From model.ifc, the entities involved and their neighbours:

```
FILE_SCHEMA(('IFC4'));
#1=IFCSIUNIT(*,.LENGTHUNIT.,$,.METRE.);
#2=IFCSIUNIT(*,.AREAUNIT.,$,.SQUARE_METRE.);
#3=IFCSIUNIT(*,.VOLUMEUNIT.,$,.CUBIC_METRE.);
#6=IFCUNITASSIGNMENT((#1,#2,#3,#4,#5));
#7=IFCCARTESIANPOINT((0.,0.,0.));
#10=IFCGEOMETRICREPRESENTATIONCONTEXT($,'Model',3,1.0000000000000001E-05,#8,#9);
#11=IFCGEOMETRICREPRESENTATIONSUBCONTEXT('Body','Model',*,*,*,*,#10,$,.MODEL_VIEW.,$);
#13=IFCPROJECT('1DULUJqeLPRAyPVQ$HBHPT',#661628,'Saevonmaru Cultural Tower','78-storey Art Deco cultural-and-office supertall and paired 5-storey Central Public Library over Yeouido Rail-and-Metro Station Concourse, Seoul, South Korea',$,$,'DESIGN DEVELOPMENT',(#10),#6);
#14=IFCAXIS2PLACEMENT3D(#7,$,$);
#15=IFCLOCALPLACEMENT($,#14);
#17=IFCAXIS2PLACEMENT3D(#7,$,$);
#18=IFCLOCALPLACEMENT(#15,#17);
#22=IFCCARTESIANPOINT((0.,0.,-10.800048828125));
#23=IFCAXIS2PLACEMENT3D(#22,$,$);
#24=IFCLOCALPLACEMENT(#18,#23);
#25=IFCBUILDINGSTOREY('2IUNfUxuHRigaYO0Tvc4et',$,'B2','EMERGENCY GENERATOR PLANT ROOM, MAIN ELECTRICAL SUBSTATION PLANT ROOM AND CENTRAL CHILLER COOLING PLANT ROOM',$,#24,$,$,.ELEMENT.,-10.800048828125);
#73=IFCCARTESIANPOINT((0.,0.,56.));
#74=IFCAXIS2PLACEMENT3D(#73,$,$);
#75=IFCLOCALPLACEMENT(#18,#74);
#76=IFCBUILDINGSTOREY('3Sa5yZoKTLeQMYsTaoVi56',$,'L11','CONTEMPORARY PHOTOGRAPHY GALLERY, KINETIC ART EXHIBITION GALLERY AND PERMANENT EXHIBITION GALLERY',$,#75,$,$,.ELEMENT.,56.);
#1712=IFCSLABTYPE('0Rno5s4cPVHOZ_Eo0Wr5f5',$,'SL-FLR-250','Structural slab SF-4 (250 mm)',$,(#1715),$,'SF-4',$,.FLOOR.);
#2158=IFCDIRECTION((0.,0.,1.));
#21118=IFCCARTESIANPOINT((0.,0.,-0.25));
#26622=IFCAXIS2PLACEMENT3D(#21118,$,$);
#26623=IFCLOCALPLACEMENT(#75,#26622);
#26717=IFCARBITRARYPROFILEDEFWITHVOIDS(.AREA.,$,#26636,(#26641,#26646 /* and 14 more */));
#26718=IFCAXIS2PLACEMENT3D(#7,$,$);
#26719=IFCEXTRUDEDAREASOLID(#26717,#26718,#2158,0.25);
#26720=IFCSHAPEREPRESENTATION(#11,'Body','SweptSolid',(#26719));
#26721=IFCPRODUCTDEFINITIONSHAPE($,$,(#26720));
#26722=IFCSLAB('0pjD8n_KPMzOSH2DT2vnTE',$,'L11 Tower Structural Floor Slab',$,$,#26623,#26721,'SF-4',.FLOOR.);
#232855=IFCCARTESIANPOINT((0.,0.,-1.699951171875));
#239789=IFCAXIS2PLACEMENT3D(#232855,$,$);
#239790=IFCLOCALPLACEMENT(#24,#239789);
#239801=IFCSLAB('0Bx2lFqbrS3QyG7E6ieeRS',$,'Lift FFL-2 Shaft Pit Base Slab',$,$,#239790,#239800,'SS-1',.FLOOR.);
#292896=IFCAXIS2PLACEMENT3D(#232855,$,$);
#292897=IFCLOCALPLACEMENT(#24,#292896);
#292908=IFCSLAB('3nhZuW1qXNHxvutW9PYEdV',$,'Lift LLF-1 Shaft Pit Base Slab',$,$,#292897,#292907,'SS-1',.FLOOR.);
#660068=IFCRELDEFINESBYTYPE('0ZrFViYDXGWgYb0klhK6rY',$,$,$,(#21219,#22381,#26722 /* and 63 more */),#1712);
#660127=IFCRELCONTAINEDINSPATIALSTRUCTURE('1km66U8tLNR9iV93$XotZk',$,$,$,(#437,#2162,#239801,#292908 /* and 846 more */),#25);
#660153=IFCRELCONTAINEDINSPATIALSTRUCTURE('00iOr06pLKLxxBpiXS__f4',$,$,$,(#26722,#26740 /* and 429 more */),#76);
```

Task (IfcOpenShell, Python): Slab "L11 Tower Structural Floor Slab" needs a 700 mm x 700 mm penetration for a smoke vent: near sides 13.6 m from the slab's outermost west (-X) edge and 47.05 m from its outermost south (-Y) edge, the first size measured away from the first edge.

```python
import numpy as np
import ifcopenshell
import ifcopenshell.api.feature
import ifcopenshell.api.geometry
import ifcopenshell.api.root
import ifcopenshell.geom
import ifcopenshell.util.placement
import ifcopenshell.util.representation
import ifcopenshell.util.shape
import ifcopenshell.util.unit

model = ifcopenshell.open("model.ifc")
unit_scale = ifcopenshell.util.unit.calculate_unit_scale(model)
settings = ifcopenshell.geom.settings()


def volume(element):
    """Net volume in cubic metres, openings subtracted."""
    shape = ifcopenshell.geom.create_shape(settings, element)
    return ifcopenshell.util.shape.get_volume(shape.geometry)


slab = model.by_guid("0pjD8n_KPMzOSH2DT2vnTE")
before = volume(slab)

# Extent in the slab's own axes, in metres. The edges named are its -X and -Y sides.
slab_shape = ifcopenshell.geom.create_shape(settings, slab)
vertices = ifcopenshell.util.shape.get_vertices(slab_shape.geometry)
x_min, y_min, bottom = vertices.min(axis=0)
top = vertices[:, 2].max()

opening = ifcopenshell.api.root.create_entity(model, ifc_class="IfcOpeningElement", name="Smoke vent opening", predefined_type="OPENING")
context = ifcopenshell.util.representation.get_context(model, "Model", "Body", "MODEL_VIEW")
width, depth = 0.7, 0.7
outline = [(0.0, 0.0), (width, 0.0), (width, depth), (0.0, depth), (0.0, 0.0)]
# Overshoot both faces by 50 mm so the cut is clean.
shape = ifcopenshell.api.geometry.add_slab_representation(
    model, context=context, depth=top - bottom + 0.1, polyline=outline
)
ifcopenshell.api.geometry.assign_representation(model, product=opening, representation=shape)

matrix = ifcopenshell.util.placement.get_local_placement(slab.ObjectPlacement)
matrix[:, 3] = matrix @ np.append(np.array([x_min + 13.6, y_min + 47.05, bottom - 0.05]) / unit_scale, 1.0)
ifcopenshell.api.geometry.edit_object_placement(model, product=opening, matrix=matrix, is_si=False)
ifcopenshell.api.feature.add_feature(model, feature=opening, element=slab)

after = volume(slab)

print(f"slab volume {before:.3f} -> {after:.3f} m3")

model.write("model_v2.ifc")
```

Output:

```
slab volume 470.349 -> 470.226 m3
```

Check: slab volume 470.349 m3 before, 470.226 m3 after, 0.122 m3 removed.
